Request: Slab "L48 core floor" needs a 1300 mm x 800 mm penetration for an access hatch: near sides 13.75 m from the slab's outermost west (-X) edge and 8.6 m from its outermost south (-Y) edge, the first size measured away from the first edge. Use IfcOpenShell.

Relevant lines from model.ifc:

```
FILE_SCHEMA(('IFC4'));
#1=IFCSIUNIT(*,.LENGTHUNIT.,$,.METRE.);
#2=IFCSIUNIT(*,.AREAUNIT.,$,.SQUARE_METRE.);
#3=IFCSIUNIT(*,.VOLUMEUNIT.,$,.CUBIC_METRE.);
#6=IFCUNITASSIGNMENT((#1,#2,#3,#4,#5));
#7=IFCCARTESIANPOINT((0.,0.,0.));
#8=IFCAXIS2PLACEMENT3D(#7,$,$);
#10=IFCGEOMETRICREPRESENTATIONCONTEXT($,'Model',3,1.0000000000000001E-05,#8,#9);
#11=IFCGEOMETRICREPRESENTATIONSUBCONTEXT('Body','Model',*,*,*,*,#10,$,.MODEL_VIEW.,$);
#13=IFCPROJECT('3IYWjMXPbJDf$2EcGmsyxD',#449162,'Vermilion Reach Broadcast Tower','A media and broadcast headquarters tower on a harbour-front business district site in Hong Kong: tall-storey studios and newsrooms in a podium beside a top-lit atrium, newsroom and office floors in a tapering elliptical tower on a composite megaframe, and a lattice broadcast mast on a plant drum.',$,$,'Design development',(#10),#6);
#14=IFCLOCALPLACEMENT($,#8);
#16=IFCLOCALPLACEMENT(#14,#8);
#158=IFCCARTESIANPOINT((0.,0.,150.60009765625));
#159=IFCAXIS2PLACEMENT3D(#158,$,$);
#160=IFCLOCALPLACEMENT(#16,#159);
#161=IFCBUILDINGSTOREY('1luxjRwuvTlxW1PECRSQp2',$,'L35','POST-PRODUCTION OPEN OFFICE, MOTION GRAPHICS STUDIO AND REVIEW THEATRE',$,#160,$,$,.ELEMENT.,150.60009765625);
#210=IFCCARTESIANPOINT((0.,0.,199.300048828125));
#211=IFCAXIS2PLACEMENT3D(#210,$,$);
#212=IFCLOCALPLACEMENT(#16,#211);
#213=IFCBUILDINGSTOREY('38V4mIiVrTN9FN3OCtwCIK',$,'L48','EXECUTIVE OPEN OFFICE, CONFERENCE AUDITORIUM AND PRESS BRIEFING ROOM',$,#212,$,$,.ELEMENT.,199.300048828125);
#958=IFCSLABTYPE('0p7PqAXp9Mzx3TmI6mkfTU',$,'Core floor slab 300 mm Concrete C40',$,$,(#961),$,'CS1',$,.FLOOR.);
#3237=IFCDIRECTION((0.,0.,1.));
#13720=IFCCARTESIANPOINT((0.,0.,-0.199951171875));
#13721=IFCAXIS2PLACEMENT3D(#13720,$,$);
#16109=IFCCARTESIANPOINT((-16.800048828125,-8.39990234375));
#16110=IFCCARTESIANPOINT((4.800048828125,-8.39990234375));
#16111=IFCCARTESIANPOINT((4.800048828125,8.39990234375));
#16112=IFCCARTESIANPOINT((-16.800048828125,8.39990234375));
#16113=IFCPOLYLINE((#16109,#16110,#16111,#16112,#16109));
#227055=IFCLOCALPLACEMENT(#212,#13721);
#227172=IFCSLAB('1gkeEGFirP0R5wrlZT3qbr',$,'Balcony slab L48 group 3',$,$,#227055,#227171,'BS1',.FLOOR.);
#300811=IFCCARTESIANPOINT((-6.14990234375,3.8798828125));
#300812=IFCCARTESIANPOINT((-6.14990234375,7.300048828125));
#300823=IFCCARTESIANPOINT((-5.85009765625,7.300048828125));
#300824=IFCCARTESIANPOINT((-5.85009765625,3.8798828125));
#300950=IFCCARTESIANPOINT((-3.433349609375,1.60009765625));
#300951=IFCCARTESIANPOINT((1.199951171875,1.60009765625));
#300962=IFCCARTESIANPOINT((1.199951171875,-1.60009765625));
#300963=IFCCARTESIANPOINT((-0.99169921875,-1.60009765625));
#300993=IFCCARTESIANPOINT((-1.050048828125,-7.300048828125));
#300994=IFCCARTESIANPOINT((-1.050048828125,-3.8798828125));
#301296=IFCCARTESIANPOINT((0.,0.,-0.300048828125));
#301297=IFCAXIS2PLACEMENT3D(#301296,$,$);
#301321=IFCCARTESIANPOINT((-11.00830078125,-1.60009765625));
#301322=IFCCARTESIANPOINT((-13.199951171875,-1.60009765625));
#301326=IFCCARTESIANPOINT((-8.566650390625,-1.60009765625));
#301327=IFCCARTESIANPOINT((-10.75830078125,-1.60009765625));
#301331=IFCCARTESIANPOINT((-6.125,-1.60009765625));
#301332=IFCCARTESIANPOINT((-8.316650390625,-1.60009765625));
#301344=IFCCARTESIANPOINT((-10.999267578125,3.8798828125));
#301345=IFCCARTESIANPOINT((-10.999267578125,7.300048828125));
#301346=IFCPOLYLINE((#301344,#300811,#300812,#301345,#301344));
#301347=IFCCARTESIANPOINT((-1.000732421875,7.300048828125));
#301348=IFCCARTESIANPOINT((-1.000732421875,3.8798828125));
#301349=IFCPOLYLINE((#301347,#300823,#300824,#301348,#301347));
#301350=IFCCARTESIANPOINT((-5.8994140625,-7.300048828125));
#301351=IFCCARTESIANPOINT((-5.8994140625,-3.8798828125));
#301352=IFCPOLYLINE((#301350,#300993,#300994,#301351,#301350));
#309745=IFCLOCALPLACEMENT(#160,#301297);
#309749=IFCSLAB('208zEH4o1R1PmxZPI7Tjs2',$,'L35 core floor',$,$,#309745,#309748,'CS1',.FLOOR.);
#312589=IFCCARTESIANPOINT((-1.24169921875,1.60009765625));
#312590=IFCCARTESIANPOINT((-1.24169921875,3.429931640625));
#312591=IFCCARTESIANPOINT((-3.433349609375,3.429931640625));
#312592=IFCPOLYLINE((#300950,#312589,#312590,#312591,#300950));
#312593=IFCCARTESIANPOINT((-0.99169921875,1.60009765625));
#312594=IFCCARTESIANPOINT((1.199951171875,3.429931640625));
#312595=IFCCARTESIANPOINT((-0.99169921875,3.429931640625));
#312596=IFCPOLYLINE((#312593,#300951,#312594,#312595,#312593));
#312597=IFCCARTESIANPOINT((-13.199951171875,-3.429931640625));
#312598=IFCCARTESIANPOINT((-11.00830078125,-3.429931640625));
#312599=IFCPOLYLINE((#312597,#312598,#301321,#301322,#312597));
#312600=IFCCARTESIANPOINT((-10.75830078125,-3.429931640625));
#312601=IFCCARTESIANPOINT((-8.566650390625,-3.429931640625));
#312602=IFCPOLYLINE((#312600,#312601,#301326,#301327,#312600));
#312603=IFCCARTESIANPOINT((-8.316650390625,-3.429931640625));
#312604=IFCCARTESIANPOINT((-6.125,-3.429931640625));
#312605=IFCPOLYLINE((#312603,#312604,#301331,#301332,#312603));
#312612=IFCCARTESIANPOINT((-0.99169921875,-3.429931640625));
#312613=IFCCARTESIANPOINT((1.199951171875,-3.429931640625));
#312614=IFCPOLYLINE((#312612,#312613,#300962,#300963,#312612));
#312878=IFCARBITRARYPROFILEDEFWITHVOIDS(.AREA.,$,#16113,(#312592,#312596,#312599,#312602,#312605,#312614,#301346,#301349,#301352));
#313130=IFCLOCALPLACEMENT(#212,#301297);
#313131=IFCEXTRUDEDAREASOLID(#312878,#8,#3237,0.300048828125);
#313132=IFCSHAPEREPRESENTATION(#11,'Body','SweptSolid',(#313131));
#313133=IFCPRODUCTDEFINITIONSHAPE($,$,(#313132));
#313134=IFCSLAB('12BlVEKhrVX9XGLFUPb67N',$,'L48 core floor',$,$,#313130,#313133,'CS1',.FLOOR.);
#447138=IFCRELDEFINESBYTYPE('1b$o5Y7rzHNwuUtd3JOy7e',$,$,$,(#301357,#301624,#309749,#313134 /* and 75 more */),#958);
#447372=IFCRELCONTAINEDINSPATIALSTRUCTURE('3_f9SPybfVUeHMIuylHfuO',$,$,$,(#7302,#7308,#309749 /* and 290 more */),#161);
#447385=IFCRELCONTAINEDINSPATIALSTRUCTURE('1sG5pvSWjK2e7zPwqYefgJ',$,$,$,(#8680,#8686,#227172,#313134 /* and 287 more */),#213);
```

```python
import numpy as np
import ifcopenshell
import ifcopenshell.api.feature
import ifcopenshell.api.geometry
import ifcopenshell.api.root
import ifcopenshell.geom
import ifcopenshell.util.placement
import ifcopenshell.util.representation
import ifcopenshell.util.shape
import ifcopenshell.util.unit

model = ifcopenshell.open("model.ifc")
unit_scale = ifcopenshell.util.unit.calculate_unit_scale(model)
settings = ifcopenshell.geom.settings()


def volume(element):
    """Net volume in cubic metres, openings subtracted."""
    shape = ifcopenshell.geom.create_shape(settings, element)
    return ifcopenshell.util.shape.get_volume(shape.geometry)


slab = model.by_guid("12BlVEKhrVX9XGLFUPb67N")
before = volume(slab)

# Extent in the slab's own axes, in metres. The edges named are its -X and -Y sides.
slab_shape = ifcopenshell.geom.create_shape(settings, slab)
vertices = ifcopenshell.util.shape.get_vertices(slab_shape.geometry)
x_min, y_min, bottom = vertices.min(axis=0)
top = vertices[:, 2].max()

opening = ifcopenshell.api.root.create_entity(model, ifc_class="IfcOpeningElement", name="Access hatch opening", predefined_type="OPENING")
context = ifcopenshell.util.representation.get_context(model, "Model", "Body", "MODEL_VIEW")
width, depth = 1.3, 0.8
outline = [(0.0, 0.0), (width, 0.0), (width, depth), (0.0, depth), (0.0, 0.0)]
# Overshoot both faces by 50 mm so the cut is clean.
shape = ifcopenshell.api.geometry.add_slab_representation(
    model, context=context, depth=top - bottom + 0.1, polyline=outline
)
ifcopenshell.api.geometry.assign_representation(model, product=opening, representation=shape)

matrix = ifcopenshell.util.placement.get_local_placement(slab.ObjectPlacement)
matrix[:, 3] = matrix @ np.append(np.array([x_min + 13.75, y_min + 8.6, bottom - 0.05]) / unit_scale, 1.0)
ifcopenshell.api.geometry.edit_object_placement(model, product=opening, matrix=matrix, is_si=False)
ifcopenshell.api.feature.add_feature(model, feature=opening, element=slab)

after = volume(slab)

print(f"slab volume {before:.3f} -> {after:.3f} m3")

model.write("model-out.ifc")
```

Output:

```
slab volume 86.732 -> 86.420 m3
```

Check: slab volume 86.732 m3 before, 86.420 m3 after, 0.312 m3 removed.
